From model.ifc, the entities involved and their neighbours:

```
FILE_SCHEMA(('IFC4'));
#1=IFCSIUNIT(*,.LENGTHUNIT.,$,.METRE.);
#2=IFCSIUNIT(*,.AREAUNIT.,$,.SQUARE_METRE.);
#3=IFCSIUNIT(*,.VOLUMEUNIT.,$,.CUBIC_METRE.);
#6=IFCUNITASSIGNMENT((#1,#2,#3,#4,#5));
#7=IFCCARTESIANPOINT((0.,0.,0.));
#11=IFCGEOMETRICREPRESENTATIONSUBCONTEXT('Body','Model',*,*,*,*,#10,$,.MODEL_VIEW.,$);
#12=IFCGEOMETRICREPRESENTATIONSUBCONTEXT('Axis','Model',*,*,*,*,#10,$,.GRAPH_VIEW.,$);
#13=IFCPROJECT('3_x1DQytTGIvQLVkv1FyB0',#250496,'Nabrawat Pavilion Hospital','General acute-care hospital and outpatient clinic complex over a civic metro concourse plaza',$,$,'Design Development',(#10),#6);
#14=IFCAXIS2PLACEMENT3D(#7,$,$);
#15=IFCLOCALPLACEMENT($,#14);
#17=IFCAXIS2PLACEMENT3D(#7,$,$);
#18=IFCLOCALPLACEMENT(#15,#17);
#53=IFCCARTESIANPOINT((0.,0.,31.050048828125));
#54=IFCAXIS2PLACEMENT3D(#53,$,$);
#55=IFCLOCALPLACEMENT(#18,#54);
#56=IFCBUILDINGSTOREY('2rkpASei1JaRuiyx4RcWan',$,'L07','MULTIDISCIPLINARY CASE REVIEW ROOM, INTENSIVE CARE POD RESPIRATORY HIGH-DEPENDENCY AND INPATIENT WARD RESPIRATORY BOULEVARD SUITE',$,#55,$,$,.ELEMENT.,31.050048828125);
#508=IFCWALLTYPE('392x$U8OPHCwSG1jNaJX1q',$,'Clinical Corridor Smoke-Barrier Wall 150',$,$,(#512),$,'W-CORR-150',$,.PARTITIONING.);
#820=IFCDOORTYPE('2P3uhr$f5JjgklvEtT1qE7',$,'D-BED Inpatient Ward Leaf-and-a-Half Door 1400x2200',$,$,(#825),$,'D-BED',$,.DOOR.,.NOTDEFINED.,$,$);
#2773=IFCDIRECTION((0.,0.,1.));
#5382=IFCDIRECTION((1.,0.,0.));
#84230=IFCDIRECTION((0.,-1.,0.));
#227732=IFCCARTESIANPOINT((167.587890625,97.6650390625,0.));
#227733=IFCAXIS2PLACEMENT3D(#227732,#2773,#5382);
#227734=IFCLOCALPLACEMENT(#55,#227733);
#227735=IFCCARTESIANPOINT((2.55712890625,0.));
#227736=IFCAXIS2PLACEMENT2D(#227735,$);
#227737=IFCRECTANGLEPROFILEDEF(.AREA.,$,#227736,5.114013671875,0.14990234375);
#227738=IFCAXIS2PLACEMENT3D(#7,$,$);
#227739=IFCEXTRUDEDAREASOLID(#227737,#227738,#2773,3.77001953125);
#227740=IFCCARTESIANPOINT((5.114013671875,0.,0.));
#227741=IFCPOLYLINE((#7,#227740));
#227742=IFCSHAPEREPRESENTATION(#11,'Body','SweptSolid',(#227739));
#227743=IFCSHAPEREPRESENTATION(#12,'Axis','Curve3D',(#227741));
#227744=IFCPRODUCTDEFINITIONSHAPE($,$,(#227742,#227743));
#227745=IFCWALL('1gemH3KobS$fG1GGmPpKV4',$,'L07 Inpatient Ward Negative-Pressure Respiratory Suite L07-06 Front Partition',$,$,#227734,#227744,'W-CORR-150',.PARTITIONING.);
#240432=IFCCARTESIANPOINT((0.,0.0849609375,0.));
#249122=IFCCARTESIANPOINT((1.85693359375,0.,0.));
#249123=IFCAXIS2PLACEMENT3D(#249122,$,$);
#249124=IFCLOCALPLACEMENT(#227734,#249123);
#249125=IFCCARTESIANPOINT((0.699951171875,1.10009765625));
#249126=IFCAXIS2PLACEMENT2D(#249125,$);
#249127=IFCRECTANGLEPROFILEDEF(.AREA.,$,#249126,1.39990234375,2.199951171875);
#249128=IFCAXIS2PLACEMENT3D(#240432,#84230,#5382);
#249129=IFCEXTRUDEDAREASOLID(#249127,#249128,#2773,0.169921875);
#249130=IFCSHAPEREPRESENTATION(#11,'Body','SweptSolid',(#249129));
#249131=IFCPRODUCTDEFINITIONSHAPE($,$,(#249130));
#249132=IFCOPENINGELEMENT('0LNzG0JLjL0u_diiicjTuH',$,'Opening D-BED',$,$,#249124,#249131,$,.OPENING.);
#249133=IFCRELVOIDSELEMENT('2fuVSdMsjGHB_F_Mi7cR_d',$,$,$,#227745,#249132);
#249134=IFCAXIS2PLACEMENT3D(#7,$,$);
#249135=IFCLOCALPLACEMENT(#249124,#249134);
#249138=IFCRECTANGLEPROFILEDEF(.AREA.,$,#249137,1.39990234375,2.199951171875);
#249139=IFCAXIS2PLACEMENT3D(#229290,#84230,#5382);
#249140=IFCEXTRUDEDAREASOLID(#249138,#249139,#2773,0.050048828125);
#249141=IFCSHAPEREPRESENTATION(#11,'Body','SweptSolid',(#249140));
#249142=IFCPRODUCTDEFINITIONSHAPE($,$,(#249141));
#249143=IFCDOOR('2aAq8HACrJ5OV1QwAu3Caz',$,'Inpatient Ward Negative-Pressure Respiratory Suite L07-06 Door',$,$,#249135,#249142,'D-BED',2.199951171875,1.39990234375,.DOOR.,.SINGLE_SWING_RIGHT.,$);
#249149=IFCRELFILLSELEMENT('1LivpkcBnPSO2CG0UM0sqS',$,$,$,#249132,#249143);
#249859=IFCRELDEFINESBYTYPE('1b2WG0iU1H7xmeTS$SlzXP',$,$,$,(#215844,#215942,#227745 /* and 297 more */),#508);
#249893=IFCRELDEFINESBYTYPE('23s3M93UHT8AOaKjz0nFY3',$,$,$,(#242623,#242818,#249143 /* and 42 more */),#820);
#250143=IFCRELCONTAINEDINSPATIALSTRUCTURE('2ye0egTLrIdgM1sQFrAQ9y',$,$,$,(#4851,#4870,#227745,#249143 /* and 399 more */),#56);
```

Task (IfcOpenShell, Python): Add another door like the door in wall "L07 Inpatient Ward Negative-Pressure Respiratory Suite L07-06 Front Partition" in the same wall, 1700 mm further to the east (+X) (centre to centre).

```python
import ifcopenshell
import ifcopenshell.api.feature
import ifcopenshell.api.geometry
import ifcopenshell.api.root
import ifcopenshell.geom
import ifcopenshell.util.element
import ifcopenshell.util.placement
import ifcopenshell.util.shape
import ifcopenshell.util.unit

model = ifcopenshell.open("model.ifc")
unit_scale = ifcopenshell.util.unit.calculate_unit_scale(model)
settings = ifcopenshell.geom.settings()


def volume(element):
    """Net volume in cubic metres, openings subtracted."""
    shape = ifcopenshell.geom.create_shape(settings, element)
    return ifcopenshell.util.shape.get_volume(shape.geometry)


door = model.by_id(249143)
opening = door.FillsVoids[0].RelatingOpeningElement
wall = opening.VoidsElements[0].RelatingBuildingElement
before = volume(wall)
shift = ifcopenshell.util.placement.get_local_placement(wall.ObjectPlacement)[:3, 0] * 1.7 / unit_scale

# copy_class copies the void relationship, type, container and properties, but no geometry.
new_opening = ifcopenshell.api.root.copy_class(model, product=opening)
new_opening.Representation = ifcopenshell.util.element.copy_deep(
    model, opening.Representation, exclude=["IfcGeometricRepresentationContext", "IfcRepresentationMap"]
)
new_door = ifcopenshell.api.root.copy_class(model, product=door)
new_door.Representation = ifcopenshell.util.element.copy_deep(
    model, door.Representation, exclude=["IfcGeometricRepresentationContext", "IfcRepresentationMap"]
)
new_door.Tag = None
ifcopenshell.api.feature.add_filling(model, opening=new_opening, element=new_door)

for old, new in ((opening, new_opening), (door, new_door)):
    matrix = ifcopenshell.util.placement.get_local_placement(old.ObjectPlacement)
    matrix[:3, 3] += shift
    ifcopenshell.api.geometry.edit_object_placement(model, product=new, matrix=matrix, is_si=False)

after = volume(wall)

print(f"wall volume {before:.3f} -> {after:.3f} m3")

model.write("model_updated.ifc")
```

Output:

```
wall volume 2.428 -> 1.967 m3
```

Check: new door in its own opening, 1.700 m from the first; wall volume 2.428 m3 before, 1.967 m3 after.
